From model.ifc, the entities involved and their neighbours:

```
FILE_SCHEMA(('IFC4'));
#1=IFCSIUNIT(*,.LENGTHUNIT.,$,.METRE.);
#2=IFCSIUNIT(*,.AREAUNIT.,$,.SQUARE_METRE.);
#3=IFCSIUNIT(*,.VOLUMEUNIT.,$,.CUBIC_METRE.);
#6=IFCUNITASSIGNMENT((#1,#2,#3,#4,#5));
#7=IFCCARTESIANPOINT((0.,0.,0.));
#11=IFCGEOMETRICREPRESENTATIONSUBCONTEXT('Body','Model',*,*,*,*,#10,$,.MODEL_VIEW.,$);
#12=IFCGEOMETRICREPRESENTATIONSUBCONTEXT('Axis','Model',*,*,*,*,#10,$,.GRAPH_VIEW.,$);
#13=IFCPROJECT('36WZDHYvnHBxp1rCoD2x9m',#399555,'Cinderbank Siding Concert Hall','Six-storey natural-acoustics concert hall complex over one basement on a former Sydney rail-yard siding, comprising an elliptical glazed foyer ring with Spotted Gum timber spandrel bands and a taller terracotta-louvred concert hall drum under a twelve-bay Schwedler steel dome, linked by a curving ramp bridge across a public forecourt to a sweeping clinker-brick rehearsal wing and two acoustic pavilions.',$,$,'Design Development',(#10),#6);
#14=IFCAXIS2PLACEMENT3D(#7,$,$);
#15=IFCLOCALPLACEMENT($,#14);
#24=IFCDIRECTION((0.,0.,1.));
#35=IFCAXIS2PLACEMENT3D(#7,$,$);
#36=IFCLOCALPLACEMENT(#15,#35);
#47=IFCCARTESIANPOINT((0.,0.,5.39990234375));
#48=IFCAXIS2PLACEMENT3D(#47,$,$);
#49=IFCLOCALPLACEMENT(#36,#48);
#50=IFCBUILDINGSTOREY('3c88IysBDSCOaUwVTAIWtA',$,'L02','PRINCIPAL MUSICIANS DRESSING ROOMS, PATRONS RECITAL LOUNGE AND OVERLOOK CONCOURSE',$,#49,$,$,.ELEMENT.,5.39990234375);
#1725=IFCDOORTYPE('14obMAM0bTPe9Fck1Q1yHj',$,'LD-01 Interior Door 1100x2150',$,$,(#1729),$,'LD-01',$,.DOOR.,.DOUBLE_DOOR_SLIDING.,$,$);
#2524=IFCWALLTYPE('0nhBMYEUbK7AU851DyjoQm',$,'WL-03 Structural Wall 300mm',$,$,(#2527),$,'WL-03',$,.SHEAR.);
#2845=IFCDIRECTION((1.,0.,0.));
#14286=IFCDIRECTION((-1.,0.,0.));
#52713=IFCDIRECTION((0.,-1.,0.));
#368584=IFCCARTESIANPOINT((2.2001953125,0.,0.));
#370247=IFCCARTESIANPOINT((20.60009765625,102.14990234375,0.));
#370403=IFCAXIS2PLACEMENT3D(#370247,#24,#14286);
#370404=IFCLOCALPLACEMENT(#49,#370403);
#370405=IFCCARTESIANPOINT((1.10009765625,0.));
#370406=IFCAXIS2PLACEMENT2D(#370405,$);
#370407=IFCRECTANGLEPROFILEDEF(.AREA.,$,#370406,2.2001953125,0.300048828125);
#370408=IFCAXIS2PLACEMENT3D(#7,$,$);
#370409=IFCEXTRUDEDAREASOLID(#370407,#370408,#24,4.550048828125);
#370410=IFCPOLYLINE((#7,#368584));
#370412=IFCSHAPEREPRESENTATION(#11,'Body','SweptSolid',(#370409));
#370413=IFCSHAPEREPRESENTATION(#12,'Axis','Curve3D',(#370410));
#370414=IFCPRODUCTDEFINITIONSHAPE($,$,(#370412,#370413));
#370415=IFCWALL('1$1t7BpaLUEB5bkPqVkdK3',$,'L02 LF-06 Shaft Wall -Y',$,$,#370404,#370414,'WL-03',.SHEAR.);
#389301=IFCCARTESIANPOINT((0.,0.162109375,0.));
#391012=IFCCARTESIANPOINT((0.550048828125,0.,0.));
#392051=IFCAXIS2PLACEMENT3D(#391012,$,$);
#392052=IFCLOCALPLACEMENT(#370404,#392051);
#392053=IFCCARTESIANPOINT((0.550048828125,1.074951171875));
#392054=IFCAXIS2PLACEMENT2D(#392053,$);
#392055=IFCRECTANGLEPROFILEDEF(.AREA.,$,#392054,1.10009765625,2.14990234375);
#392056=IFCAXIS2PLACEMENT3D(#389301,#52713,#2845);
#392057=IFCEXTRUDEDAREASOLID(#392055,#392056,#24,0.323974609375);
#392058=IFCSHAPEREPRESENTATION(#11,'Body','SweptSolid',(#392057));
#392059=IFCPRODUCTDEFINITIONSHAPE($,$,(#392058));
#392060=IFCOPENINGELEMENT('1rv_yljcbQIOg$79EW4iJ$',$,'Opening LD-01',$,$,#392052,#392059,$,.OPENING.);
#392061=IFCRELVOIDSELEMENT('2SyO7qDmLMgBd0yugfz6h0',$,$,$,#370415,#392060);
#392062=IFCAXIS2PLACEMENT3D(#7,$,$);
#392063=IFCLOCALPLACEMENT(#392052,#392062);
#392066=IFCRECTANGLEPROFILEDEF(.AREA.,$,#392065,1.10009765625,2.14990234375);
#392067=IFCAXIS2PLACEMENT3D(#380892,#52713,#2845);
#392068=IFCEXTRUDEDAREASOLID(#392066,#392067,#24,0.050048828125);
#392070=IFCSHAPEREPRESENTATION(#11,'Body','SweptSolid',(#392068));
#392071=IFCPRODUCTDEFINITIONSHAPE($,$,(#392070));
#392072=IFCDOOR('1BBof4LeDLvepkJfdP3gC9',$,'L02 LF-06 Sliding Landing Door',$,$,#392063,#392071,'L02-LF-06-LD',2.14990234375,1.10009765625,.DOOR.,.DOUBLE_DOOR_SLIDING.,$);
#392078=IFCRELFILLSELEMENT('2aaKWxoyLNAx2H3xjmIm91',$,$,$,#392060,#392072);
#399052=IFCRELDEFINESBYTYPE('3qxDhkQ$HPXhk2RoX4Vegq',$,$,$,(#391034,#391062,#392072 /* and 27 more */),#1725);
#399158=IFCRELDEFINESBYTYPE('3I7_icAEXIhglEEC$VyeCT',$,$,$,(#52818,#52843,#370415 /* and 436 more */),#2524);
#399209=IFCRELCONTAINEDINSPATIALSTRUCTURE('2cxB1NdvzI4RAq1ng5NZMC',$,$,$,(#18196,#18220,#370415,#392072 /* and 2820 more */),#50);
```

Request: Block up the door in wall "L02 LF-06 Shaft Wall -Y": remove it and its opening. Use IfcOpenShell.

```python
import ifcopenshell
import ifcopenshell.api.feature
import ifcopenshell.api.root
import ifcopenshell.geom
import ifcopenshell.util.shape

model = ifcopenshell.open("model.ifc")
settings = ifcopenshell.geom.settings()


def volume(element):
    """Net volume in cubic metres, openings subtracted."""
    shape = ifcopenshell.geom.create_shape(settings, element)
    return ifcopenshell.util.shape.get_volume(shape.geometry)


door = model.by_guid("1BBof4LeDLvepkJfdP3gC9")
opening = door.FillsVoids[0].RelatingOpeningElement
wall = opening.VoidsElements[0].RelatingBuildingElement
before = volume(wall)

ifcopenshell.api.root.remove_product(model, product=door)
ifcopenshell.api.feature.remove_feature(model, feature=opening)

after = volume(wall)

print(f"wall volume {before:.3f} -> {after:.3f} m3")

model.write("model_v2.ifc")
```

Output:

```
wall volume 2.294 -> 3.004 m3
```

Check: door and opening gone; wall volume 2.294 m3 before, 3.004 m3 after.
